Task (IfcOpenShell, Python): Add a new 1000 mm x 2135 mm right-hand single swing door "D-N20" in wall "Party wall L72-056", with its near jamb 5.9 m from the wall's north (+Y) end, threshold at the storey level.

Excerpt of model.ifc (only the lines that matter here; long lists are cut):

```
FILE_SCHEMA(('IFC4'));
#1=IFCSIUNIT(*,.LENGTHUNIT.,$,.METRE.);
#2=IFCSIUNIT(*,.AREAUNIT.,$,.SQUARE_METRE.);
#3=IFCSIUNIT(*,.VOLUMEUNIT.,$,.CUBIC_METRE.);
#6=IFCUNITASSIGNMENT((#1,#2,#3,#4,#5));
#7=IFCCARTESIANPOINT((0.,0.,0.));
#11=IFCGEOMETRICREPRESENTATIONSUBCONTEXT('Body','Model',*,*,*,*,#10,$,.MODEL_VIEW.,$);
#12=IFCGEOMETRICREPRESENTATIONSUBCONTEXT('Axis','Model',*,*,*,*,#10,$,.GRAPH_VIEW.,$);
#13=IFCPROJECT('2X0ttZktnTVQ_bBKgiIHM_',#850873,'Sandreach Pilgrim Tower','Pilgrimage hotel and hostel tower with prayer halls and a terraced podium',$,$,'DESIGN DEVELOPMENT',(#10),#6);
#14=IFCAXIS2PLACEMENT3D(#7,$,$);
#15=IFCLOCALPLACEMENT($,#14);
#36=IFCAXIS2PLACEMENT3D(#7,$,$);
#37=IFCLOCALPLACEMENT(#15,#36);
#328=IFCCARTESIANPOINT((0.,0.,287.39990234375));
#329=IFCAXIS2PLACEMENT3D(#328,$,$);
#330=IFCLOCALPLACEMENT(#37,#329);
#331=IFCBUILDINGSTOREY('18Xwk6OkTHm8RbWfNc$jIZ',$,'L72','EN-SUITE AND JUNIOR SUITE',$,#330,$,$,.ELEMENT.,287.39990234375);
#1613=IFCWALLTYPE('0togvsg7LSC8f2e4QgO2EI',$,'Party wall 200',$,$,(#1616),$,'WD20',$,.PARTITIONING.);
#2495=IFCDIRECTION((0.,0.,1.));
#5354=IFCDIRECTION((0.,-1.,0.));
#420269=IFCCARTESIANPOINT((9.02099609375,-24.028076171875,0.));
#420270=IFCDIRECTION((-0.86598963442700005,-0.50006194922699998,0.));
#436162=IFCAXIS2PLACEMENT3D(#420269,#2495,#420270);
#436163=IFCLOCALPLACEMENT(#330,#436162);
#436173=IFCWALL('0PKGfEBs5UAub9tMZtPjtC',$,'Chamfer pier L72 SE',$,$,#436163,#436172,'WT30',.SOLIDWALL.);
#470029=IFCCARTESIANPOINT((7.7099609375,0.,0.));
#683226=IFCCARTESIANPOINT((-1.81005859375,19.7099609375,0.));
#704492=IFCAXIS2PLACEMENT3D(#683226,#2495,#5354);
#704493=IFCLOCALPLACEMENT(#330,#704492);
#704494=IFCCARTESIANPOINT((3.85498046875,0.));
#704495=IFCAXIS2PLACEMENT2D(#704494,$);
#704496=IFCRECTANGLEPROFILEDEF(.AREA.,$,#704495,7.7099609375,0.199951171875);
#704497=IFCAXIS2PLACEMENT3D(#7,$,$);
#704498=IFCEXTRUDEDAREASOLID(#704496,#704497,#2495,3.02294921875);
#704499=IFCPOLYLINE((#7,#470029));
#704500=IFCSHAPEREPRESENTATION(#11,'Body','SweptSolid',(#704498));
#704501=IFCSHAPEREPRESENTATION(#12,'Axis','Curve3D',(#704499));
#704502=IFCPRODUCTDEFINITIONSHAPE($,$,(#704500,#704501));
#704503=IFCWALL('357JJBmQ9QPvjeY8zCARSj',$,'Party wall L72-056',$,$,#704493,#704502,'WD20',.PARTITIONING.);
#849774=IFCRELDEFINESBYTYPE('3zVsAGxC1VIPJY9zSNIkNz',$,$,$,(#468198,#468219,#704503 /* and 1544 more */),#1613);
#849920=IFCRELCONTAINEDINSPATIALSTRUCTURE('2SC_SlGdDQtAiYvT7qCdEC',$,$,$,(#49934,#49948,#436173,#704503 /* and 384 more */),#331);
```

```python
import numpy as np
import ifcopenshell
import ifcopenshell.api.feature
import ifcopenshell.api.geometry
import ifcopenshell.api.root
import ifcopenshell.api.spatial
import ifcopenshell.geom
import ifcopenshell.util.element
import ifcopenshell.util.placement
import ifcopenshell.util.representation
import ifcopenshell.util.shape
import ifcopenshell.util.unit

model = ifcopenshell.open("model.ifc")
unit_scale = ifcopenshell.util.unit.calculate_unit_scale(model)
settings = ifcopenshell.geom.settings()


def volume(element):
    """Net volume in cubic metres, openings subtracted."""
    shape = ifcopenshell.geom.create_shape(settings, element)
    return ifcopenshell.util.shape.get_volume(shape.geometry)


wall = model.by_guid("357JJBmQ9QPvjeY8zCARSj")
storey = ifcopenshell.util.element.get_container(wall, ifc_class="IfcBuildingStorey")
context = ifcopenshell.util.representation.get_context(model, "Model", "Body", "MODEL_VIEW")
before = volume(wall)

width, height, from_end, sill = 1, 2.135, 5.9, 0.0  # metres

# The wall runs along its own X axis, and the end named is its -X end.
wall_shape = ifcopenshell.geom.create_shape(settings, wall)
x, y, z = ifcopenshell.util.shape.get_vertices(wall_shape.geometry).T
start = x.min() + from_end
face, thickness = float(y.min()), float(y.max() - y.min())
wall_matrix = ifcopenshell.util.placement.get_local_placement(wall.ObjectPlacement)
level = ifcopenshell.util.placement.get_local_placement(storey.ObjectPlacement)[2, 3]


def in_wall(x, y):
    """Placement at x, y metres in the wall's axes, at sill height."""
    matrix = wall_matrix.copy()
    matrix[:, 3] = wall_matrix @ np.array([x / unit_scale, y / unit_scale, 0.0, 1.0])
    matrix[2, 3] = level + sill / unit_scale
    return matrix


# Opening: a box that overshoots both wall faces by 50 mm.
opening = ifcopenshell.api.root.create_entity(model, ifc_class="IfcOpeningElement", predefined_type="OPENING")
box = ifcopenshell.api.geometry.add_wall_representation(
    model, context=context, length=width, height=height, thickness=thickness + 0.1
)
ifcopenshell.api.geometry.assign_representation(model, product=opening, representation=box)
ifcopenshell.api.geometry.edit_object_placement(model, product=opening, matrix=in_wall(start, face - 0.05), is_si=False)
ifcopenshell.api.feature.add_feature(model, feature=opening, element=wall)

door = ifcopenshell.api.root.create_entity(model, ifc_class="IfcDoor", name="D-N20", predefined_type="DOOR")
door.OverallWidth, door.OverallHeight = width / unit_scale, height / unit_scale
door.OperationType = "SINGLE_SWING_RIGHT"
body = ifcopenshell.api.geometry.add_door_representation(
    model,
    context=context,
    overall_width=door.OverallWidth,
    overall_height=door.OverallHeight,
    operation_type="SINGLE_SWING_RIGHT",
    lining_properties={"LiningDepth": thickness / unit_scale, "ThresholdDepth": thickness / unit_scale},
)
ifcopenshell.api.geometry.assign_representation(model, product=door, representation=body)
ifcopenshell.api.spatial.assign_container(model, products=[door], relating_structure=storey)
ifcopenshell.api.feature.add_filling(model, opening=opening, element=door)

# The lining spans the wall, so the door starts at the wall face.
ifcopenshell.api.geometry.edit_object_placement(model, product=door, matrix=in_wall(start, face), is_si=False)

after = volume(wall)

print(f"wall volume {before:.3f} -> {after:.3f} m3")

model.write("model_updated.ifc")
```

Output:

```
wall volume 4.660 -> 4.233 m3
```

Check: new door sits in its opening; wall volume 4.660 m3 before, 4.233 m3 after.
